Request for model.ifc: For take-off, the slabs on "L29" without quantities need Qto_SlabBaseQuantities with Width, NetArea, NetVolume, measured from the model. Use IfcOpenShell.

First a look at what the model holds.

```python
import ifcopenshell
import ifcopenshell.util.element
import ifcopenshell.util.unit

model = ifcopenshell.open("model.ifc")
print(model.schema)
for unit_type in ("LENGTHUNIT", "AREAUNIT", "VOLUMEUNIT"):
    print(unit_type, ifcopenshell.util.unit.calculate_unit_scale(model, unit_type))
storey = next(s for s in model.by_type("IfcBuildingStorey") if s.Name == "L29")
slabs = [e for e in ifcopenshell.util.element.get_decomposition(storey) if e.is_a("IfcSlab")]
for e in sorted(slabs, key=lambda e: e.id()):
    print(e.id(), e.is_a(), e.Name, list(ifcopenshell.util.element.get_psets(e, qtos_only=True)), sep=" | ")
```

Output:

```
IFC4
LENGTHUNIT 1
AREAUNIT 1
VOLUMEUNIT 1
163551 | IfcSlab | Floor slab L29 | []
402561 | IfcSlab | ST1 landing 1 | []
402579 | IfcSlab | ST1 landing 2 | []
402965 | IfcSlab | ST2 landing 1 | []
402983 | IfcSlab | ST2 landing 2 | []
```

```python
import ifcopenshell
import ifcopenshell.api.pset
import ifcopenshell.geom
import ifcopenshell.util.element
import ifcopenshell.util.shape
import ifcopenshell.util.unit

model = ifcopenshell.open("model.ifc")
unit_scale = ifcopenshell.util.unit.calculate_unit_scale(model)
area_scale = ifcopenshell.util.unit.calculate_unit_scale(model, "AREAUNIT")
volume_scale = ifcopenshell.util.unit.calculate_unit_scale(model, "VOLUMEUNIT")
settings = ifcopenshell.geom.settings()

storey = next(s for s in model.by_type("IfcBuildingStorey") if s.Name == "L29")
slabs = [e for e in ifcopenshell.util.element.get_decomposition(storey) if e.is_a("IfcSlab")]

for e in sorted(slabs, key=lambda e: e.id()):
    if ifcopenshell.util.element.get_psets(e, qtos_only=True, should_inherit=False):
        continue
    # Geometry comes back in metres, in the element's own axes.
    shape = ifcopenshell.geom.create_shape(settings, e)
    values = {
        "Width": ifcopenshell.util.shape.get_z(shape.geometry) / unit_scale,
        "NetArea": ifcopenshell.util.shape.get_footprint_area(shape.geometry) / area_scale,
        "NetVolume": ifcopenshell.util.shape.get_volume(shape.geometry) / volume_scale,
    }
    qto = ifcopenshell.api.pset.add_qto(model, product=e, name="Qto_SlabBaseQuantities")
    ifcopenshell.api.pset.edit_qto(model, qto=qto, properties=values)
    print(e.id(), {k: round(v, 3) for k, v in values.items()})

model.write("model_edited.ifc")
```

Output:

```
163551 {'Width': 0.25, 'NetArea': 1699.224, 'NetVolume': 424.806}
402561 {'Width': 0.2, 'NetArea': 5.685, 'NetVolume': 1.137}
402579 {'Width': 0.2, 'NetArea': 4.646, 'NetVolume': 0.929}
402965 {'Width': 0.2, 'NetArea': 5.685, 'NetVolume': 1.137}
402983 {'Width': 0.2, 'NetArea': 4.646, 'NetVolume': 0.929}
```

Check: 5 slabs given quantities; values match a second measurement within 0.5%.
